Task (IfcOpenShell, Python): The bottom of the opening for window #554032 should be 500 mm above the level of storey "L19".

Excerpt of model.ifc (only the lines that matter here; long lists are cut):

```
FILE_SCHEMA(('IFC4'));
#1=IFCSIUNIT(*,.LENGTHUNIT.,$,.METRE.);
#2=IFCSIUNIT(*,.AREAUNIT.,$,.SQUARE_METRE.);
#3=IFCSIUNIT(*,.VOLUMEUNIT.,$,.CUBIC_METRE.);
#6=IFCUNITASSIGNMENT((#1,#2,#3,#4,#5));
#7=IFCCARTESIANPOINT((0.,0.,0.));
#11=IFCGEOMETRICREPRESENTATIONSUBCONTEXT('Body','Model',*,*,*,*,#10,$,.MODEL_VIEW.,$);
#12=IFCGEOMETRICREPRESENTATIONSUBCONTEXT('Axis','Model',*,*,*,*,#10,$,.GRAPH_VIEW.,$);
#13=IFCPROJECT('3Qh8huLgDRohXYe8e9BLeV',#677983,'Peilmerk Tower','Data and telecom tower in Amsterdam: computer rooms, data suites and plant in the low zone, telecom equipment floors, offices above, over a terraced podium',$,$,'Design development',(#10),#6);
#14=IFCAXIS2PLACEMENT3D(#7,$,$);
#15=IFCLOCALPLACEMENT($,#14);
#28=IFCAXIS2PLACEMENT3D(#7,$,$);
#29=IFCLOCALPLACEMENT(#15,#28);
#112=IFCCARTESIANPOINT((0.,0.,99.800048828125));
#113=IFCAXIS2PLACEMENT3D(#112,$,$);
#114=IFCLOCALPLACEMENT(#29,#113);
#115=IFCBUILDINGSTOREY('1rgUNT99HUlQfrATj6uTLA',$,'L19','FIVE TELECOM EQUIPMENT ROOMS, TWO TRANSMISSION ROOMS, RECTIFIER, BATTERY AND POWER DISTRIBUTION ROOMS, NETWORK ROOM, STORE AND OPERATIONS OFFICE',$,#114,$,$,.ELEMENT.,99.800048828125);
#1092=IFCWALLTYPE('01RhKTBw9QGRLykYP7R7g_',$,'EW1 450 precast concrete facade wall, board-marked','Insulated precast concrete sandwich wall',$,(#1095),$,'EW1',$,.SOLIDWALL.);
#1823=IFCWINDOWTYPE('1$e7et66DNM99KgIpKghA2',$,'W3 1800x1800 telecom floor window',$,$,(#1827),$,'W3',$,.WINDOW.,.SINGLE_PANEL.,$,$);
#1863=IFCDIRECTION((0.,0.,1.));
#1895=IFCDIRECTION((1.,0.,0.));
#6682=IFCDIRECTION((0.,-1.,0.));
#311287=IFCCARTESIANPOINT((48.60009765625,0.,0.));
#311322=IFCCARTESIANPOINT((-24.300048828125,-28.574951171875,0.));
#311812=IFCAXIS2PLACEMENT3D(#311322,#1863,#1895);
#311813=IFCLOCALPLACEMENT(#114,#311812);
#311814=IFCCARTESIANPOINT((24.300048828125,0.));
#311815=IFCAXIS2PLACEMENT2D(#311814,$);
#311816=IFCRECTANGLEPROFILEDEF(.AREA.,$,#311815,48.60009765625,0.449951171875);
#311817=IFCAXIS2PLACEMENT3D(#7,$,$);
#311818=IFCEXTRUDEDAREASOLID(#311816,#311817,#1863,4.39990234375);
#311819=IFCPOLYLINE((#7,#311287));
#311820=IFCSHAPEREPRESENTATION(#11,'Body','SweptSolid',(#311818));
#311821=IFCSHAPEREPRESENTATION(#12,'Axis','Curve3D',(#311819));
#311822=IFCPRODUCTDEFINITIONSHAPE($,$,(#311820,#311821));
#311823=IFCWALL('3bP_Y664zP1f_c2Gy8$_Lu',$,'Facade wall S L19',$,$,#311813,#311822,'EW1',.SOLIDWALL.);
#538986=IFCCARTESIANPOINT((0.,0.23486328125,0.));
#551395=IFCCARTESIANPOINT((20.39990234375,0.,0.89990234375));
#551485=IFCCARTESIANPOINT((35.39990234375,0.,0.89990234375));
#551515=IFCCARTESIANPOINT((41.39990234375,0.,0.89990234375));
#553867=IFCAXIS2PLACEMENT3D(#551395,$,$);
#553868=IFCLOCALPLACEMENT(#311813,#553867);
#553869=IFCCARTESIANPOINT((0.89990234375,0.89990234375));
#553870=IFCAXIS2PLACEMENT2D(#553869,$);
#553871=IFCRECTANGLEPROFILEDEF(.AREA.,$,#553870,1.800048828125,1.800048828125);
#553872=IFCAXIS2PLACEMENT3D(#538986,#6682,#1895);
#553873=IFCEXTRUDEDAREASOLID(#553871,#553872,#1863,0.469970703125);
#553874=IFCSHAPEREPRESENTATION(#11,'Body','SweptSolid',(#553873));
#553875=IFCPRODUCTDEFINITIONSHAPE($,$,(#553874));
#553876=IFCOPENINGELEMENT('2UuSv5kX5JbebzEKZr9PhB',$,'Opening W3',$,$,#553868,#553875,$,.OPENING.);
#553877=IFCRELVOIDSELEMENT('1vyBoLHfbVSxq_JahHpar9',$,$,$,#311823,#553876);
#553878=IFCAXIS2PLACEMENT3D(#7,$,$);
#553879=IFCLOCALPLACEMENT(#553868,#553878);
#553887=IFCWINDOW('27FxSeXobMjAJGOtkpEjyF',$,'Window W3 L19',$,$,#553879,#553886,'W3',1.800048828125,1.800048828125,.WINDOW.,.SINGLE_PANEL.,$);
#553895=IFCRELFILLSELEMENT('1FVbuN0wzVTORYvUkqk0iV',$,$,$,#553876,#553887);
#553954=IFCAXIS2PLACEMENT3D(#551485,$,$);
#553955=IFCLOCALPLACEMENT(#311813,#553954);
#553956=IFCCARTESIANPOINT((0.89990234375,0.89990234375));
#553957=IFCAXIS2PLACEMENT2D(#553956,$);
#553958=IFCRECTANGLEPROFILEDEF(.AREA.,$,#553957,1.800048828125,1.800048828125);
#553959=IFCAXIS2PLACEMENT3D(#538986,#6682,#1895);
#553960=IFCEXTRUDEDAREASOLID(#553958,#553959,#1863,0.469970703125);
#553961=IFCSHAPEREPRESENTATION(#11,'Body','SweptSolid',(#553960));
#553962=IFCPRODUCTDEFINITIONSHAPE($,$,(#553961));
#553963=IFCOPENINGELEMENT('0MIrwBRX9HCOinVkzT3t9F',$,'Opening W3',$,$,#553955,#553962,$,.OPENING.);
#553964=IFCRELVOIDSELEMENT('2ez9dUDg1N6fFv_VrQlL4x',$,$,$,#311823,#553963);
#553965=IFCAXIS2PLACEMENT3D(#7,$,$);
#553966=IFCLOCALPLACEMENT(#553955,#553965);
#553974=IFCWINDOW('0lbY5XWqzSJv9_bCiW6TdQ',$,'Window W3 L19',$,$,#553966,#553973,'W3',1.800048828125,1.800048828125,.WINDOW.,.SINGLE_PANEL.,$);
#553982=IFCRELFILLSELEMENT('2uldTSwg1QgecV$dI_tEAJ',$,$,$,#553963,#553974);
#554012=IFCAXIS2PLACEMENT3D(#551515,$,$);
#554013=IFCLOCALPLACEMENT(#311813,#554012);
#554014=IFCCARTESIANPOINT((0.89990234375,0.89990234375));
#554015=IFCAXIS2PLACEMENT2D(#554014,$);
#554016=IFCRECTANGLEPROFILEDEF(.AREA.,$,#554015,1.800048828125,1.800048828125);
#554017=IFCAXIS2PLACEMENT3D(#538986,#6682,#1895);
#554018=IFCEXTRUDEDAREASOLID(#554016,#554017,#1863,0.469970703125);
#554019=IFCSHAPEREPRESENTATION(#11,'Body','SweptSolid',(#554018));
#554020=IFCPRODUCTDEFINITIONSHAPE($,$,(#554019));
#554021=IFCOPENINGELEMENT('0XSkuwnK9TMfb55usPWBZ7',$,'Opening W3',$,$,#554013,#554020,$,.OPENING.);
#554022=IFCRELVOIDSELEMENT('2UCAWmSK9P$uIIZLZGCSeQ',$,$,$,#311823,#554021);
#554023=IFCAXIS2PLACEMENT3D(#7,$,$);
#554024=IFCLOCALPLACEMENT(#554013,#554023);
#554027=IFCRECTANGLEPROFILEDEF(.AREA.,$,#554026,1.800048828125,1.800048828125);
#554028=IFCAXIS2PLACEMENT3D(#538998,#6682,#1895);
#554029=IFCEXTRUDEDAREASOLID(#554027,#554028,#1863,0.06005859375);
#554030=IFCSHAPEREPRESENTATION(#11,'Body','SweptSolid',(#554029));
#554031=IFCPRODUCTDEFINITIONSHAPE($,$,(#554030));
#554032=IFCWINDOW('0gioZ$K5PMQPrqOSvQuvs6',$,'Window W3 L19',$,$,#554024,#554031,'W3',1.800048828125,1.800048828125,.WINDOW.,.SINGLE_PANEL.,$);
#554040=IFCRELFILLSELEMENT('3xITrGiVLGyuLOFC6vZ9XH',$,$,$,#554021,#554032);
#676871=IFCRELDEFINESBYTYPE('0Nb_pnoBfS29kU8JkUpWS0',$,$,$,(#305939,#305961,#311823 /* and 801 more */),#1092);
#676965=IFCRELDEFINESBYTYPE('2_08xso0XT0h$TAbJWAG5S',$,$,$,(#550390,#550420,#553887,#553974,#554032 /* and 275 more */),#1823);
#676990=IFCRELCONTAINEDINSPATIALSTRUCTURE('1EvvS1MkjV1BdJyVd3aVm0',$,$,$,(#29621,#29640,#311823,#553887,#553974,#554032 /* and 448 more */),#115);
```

```python
import numpy as np
import ifcopenshell
import ifcopenshell.api.geometry
import ifcopenshell.geom
import ifcopenshell.util.element
import ifcopenshell.util.placement
import ifcopenshell.util.shape
import ifcopenshell.util.unit

model = ifcopenshell.open("model.ifc")
unit_scale = ifcopenshell.util.unit.calculate_unit_scale(model)

window = model.by_guid("0gioZ$K5PMQPrqOSvQuvs6")
opening = window.FillsVoids[0].RelatingOpeningElement
storey = ifcopenshell.util.element.get_container(window, ifc_class="IfcBuildingStorey")
level = ifcopenshell.util.placement.get_local_placement(storey.ObjectPlacement)[2, 3]

# The opening's origin need not be at the sill, so measure its lowest point.
shape = ifcopenshell.geom.create_shape(ifcopenshell.geom.settings(), opening)
bottom = ifcopenshell.util.shape.get_shape_bottom_elevation(shape, shape.geometry) / unit_scale
dz = level + 0.5 / unit_scale - bottom

shift = np.array([0.0, 0.0, dz])
# The window is placed relative to its opening, so it follows when the opening moves.
matrix = ifcopenshell.util.placement.get_local_placement(opening.ObjectPlacement)
matrix[:3, 3] += shift
ifcopenshell.api.geometry.edit_object_placement(
    model, product=opening, matrix=matrix, is_si=False, should_transform_children=True
)

print(f"moved by {dz * unit_scale:+.3f} m")

model.write("model_edited.ifc")
```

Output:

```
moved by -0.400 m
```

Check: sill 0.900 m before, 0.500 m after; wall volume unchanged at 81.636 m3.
